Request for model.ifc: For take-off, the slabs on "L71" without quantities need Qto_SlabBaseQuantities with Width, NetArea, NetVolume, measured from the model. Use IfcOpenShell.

First a look at what the model holds.

```python
import ifcopenshell
import ifcopenshell.util.element
import ifcopenshell.util.unit

model = ifcopenshell.open("model.ifc")
print(model.schema)
for unit_type in ("LENGTHUNIT", "AREAUNIT", "VOLUMEUNIT"):
    print(unit_type, ifcopenshell.util.unit.calculate_unit_scale(model, unit_type))
storey = next(s for s in model.by_type("IfcBuildingStorey") if s.Name == "L71")
slabs = [e for e in ifcopenshell.util.element.get_decomposition(storey) if e.is_a("IfcSlab")]
for e in sorted(slabs, key=lambda e: e.id()):
    print(e.id(), e.is_a(), e.Name, list(ifcopenshell.util.element.get_psets(e, qtos_only=True)), sep=" | ")
```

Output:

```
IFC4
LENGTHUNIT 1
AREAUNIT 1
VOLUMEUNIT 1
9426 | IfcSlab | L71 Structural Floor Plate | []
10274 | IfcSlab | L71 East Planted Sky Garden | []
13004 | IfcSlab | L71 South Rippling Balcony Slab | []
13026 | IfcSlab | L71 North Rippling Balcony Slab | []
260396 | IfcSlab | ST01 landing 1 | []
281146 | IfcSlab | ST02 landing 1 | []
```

```python
import ifcopenshell
import ifcopenshell.api.pset
import ifcopenshell.geom
import ifcopenshell.util.element
import ifcopenshell.util.shape
import ifcopenshell.util.unit

model = ifcopenshell.open("model.ifc")
unit_scale = ifcopenshell.util.unit.calculate_unit_scale(model)
area_scale = ifcopenshell.util.unit.calculate_unit_scale(model, "AREAUNIT")
volume_scale = ifcopenshell.util.unit.calculate_unit_scale(model, "VOLUMEUNIT")
settings = ifcopenshell.geom.settings()

storey = next(s for s in model.by_type("IfcBuildingStorey") if s.Name == "L71")
slabs = [e for e in ifcopenshell.util.element.get_decomposition(storey) if e.is_a("IfcSlab")]

for e in sorted(slabs, key=lambda e: e.id()):
    if ifcopenshell.util.element.get_psets(e, qtos_only=True, should_inherit=False):
        continue
    # Geometry comes back in metres, in the element's own axes.
    shape = ifcopenshell.geom.create_shape(settings, e)
    values = {
        "Width": ifcopenshell.util.shape.get_z(shape.geometry) / unit_scale,
        "NetArea": ifcopenshell.util.shape.get_footprint_area(shape.geometry) / area_scale,
        "NetVolume": ifcopenshell.util.shape.get_volume(shape.geometry) / volume_scale,
    }
    qto = ifcopenshell.api.pset.add_qto(model, product=e, name="Qto_SlabBaseQuantities")
    ifcopenshell.api.pset.edit_qto(model, qto=qto, properties=values)
    print(e.id(), {k: round(v, 3) for k, v in values.items()})

model.write("model-out.ifc")
```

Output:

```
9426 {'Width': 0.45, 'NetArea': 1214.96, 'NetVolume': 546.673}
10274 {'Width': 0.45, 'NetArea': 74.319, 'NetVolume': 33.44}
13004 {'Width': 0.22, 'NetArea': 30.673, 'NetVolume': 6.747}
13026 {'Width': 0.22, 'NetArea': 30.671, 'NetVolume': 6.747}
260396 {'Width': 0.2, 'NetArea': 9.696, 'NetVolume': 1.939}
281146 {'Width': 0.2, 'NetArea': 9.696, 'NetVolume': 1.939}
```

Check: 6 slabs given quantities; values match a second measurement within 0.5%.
